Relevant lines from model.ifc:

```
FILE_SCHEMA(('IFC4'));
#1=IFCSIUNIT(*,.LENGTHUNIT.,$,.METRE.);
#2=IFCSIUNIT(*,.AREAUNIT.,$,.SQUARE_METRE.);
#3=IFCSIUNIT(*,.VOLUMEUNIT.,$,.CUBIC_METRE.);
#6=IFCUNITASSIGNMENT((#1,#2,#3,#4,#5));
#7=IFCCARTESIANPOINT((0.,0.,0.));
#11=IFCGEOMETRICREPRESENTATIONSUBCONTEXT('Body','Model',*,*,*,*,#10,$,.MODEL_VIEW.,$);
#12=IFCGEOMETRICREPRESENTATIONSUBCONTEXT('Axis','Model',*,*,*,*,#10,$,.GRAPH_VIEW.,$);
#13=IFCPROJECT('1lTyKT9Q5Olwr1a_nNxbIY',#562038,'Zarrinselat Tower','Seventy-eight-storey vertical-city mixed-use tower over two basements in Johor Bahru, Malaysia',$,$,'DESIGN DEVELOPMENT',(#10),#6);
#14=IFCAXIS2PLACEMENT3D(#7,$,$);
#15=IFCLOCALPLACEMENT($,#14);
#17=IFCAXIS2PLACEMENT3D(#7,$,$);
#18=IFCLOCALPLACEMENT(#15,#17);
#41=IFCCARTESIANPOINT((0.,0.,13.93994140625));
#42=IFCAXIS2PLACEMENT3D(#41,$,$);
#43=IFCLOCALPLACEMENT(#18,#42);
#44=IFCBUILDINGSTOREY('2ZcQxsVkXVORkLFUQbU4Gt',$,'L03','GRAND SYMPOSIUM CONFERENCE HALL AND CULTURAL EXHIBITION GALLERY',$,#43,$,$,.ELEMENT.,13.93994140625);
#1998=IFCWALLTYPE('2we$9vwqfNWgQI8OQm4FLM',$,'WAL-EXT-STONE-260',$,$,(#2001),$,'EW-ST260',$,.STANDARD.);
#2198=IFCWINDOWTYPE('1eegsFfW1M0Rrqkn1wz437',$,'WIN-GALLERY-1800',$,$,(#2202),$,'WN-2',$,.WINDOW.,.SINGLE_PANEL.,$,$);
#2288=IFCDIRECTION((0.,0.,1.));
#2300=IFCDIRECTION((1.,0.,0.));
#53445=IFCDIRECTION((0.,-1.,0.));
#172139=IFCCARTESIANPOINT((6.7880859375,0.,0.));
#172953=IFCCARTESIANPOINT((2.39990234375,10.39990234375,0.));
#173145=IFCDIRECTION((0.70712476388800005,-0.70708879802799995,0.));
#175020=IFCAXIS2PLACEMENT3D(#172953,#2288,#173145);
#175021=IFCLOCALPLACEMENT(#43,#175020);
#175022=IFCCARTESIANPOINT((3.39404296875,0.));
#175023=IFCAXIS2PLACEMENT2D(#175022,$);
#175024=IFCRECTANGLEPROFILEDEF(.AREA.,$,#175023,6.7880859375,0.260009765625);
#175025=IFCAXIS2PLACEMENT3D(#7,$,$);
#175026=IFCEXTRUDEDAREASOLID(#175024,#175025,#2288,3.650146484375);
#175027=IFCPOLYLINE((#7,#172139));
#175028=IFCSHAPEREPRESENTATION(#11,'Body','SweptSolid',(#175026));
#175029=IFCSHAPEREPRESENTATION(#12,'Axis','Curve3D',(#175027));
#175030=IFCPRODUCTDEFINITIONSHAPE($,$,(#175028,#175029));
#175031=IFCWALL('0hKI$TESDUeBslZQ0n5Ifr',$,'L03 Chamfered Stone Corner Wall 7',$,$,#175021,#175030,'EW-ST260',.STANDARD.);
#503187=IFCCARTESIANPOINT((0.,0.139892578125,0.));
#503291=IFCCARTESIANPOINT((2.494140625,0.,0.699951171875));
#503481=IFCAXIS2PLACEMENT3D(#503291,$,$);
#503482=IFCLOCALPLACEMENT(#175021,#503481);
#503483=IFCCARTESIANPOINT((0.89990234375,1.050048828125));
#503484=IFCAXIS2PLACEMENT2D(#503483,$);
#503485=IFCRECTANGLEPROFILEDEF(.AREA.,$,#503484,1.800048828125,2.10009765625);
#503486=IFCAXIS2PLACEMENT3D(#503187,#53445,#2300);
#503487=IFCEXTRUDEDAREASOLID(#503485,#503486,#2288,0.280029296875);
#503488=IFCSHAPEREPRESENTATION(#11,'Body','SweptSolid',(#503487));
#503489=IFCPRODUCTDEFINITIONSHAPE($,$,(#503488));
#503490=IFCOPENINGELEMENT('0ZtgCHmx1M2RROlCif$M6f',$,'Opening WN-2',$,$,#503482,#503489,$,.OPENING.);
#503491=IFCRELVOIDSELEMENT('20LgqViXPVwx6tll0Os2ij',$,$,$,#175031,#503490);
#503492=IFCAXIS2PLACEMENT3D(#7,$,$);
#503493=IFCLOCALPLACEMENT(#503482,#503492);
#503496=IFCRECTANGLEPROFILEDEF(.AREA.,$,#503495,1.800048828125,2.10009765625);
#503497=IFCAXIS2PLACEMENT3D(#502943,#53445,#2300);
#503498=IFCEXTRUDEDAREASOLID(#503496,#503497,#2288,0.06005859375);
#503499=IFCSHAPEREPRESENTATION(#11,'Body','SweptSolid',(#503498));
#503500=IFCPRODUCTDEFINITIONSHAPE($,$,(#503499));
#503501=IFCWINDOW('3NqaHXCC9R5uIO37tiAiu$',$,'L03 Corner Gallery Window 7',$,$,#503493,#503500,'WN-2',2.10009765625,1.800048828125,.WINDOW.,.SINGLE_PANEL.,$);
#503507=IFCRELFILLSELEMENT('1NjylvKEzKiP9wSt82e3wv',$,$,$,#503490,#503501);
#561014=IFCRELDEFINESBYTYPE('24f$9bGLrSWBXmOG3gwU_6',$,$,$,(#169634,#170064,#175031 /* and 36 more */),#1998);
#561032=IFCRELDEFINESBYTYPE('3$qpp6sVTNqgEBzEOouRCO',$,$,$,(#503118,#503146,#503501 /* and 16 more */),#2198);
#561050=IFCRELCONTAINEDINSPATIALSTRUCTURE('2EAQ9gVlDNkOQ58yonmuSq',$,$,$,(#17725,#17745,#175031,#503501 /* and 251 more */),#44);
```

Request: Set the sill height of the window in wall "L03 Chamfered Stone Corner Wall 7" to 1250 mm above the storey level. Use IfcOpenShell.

```python
import numpy as np
import ifcopenshell
import ifcopenshell.api.geometry
import ifcopenshell.geom
import ifcopenshell.util.element
import ifcopenshell.util.placement
import ifcopenshell.util.shape
import ifcopenshell.util.unit

model = ifcopenshell.open("model.ifc")
unit_scale = ifcopenshell.util.unit.calculate_unit_scale(model)

window = model.by_id(503501)
opening = window.FillsVoids[0].RelatingOpeningElement
storey = ifcopenshell.util.element.get_container(window, ifc_class="IfcBuildingStorey")
level = ifcopenshell.util.placement.get_local_placement(storey.ObjectPlacement)[2, 3]

# The opening's origin need not be at the sill, so measure its lowest point.
shape = ifcopenshell.geom.create_shape(ifcopenshell.geom.settings(), opening)
bottom = ifcopenshell.util.shape.get_shape_bottom_elevation(shape, shape.geometry) / unit_scale
dz = level + 1.25 - bottom

shift = np.array([0.0, 0.0, dz])
# The window is placed relative to its opening, so it follows when the opening moves.
matrix = ifcopenshell.util.placement.get_local_placement(opening.ObjectPlacement)
matrix[:3, 3] += shift
ifcopenshell.api.geometry.edit_object_placement(
    model, product=opening, matrix=matrix, is_si=False, should_transform_children=True
)

print(f"moved by {dz * unit_scale:+.3f} m")

model.write("model_updated.ifc")
```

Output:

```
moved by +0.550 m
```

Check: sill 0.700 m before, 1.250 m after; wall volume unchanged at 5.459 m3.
